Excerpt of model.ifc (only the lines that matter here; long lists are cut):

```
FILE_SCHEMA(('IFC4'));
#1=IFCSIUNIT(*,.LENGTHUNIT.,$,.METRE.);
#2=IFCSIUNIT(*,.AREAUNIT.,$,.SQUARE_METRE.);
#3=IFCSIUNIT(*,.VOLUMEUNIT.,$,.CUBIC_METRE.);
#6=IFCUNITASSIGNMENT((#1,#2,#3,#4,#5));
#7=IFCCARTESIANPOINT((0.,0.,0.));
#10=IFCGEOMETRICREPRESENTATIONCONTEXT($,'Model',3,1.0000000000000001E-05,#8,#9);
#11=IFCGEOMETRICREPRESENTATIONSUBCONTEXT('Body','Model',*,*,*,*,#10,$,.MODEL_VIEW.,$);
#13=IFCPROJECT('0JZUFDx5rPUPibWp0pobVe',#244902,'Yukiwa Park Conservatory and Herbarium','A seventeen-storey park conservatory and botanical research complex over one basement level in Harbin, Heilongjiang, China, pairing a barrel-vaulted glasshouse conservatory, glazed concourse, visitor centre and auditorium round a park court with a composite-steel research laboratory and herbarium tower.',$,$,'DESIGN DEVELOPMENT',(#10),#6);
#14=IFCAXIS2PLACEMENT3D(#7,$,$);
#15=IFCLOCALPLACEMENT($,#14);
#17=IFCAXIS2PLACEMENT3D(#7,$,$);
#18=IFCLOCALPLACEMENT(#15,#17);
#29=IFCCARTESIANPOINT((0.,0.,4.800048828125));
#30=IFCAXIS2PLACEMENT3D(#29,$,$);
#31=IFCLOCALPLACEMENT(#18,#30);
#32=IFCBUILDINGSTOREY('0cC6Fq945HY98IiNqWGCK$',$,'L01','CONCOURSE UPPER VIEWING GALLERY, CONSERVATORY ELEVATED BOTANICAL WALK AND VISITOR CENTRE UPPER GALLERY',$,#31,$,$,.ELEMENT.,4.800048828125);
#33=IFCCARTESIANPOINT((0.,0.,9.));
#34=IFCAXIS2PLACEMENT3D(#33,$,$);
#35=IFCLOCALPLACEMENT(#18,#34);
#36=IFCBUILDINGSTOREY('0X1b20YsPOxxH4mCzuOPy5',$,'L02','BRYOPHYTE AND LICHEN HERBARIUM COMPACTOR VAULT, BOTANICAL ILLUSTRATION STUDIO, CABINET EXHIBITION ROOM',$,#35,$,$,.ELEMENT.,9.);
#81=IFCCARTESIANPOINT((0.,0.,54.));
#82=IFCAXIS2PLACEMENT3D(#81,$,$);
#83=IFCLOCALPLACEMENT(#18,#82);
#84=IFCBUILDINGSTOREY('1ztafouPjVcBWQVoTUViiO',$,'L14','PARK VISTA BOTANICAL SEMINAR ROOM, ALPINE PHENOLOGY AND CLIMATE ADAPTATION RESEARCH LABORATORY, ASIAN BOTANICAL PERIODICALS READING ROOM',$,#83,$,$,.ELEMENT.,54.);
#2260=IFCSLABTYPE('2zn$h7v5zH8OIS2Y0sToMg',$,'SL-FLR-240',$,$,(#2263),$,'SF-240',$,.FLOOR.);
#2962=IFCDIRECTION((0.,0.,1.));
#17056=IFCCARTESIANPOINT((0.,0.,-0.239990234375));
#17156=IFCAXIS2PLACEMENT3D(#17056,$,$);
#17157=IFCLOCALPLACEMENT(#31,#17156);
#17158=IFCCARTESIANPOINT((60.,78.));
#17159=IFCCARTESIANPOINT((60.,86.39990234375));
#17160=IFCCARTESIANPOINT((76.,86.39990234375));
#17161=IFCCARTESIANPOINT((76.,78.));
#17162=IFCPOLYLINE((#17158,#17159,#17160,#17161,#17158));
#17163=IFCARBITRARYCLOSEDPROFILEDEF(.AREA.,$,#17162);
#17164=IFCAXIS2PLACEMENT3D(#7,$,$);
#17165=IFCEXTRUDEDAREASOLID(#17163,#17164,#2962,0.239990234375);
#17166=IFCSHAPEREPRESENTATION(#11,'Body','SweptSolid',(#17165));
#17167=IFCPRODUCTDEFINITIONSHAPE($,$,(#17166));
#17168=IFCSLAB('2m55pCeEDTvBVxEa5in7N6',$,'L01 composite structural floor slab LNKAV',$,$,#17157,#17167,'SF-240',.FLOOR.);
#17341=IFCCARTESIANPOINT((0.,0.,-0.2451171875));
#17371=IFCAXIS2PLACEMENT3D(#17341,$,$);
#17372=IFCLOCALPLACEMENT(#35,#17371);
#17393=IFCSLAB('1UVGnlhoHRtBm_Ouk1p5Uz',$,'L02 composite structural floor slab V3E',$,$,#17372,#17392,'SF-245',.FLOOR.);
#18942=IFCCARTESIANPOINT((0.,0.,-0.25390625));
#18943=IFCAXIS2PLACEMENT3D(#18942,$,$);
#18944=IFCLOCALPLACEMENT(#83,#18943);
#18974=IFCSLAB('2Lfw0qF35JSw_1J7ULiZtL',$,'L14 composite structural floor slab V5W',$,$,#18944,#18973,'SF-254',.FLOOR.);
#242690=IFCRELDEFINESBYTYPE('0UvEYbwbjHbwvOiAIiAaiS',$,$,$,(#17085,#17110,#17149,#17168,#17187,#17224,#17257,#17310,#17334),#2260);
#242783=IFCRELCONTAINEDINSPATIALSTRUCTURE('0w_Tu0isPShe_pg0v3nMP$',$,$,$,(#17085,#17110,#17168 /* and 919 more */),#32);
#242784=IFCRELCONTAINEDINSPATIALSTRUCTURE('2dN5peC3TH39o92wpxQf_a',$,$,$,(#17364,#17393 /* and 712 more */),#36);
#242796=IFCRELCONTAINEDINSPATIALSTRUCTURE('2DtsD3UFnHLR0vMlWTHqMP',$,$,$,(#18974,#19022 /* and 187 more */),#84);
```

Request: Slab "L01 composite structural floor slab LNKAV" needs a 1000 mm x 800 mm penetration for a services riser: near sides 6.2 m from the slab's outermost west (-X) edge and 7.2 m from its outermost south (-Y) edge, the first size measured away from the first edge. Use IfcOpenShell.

```python
import numpy as np
import ifcopenshell
import ifcopenshell.api.feature
import ifcopenshell.api.geometry
import ifcopenshell.api.root
import ifcopenshell.geom
import ifcopenshell.util.placement
import ifcopenshell.util.representation
import ifcopenshell.util.shape
import ifcopenshell.util.unit

model = ifcopenshell.open("model.ifc")
unit_scale = ifcopenshell.util.unit.calculate_unit_scale(model)
settings = ifcopenshell.geom.settings()


def volume(element):
    """Net volume in cubic metres, openings subtracted."""
    shape = ifcopenshell.geom.create_shape(settings, element)
    return ifcopenshell.util.shape.get_volume(shape.geometry)


slab = model.by_guid("2m55pCeEDTvBVxEa5in7N6")
before = volume(slab)

# Extent in the slab's own axes, in metres. The edges named are its -X and -Y sides.
slab_shape = ifcopenshell.geom.create_shape(settings, slab)
vertices = ifcopenshell.util.shape.get_vertices(slab_shape.geometry)
x_min, y_min, bottom = vertices.min(axis=0)
top = vertices[:, 2].max()

opening = ifcopenshell.api.root.create_entity(model, ifc_class="IfcOpeningElement", name="Services riser opening", predefined_type="OPENING")
context = ifcopenshell.util.representation.get_context(model, "Model", "Body", "MODEL_VIEW")
width, depth = 1, 0.8
outline = [(0.0, 0.0), (width, 0.0), (width, depth), (0.0, depth), (0.0, 0.0)]
# Overshoot both faces by 50 mm so the cut is clean.
shape = ifcopenshell.api.geometry.add_slab_representation(
    model, context=context, depth=top - bottom + 0.1, polyline=outline
)
ifcopenshell.api.geometry.assign_representation(model, product=opening, representation=shape)

matrix = ifcopenshell.util.placement.get_local_placement(slab.ObjectPlacement)
matrix[:, 3] = matrix @ np.append(np.array([x_min + 6.2, y_min + 7.2, bottom - 0.05]) / unit_scale, 1.0)
ifcopenshell.api.geometry.edit_object_placement(model, product=opening, matrix=matrix, is_si=False)
ifcopenshell.api.feature.add_feature(model, feature=opening, element=slab)

after = volume(slab)

print(f"slab volume {before:.3f} -> {after:.3f} m3")

model.write("model_updated.ifc")
```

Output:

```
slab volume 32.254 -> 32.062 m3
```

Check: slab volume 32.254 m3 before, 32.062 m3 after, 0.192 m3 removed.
